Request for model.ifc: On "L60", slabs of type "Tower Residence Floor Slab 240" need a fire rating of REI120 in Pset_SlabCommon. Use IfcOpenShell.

First a look at what the model holds.

```python
import ifcopenshell
import ifcopenshell.util.element

model = ifcopenshell.open("model.ifc")
print(model.schema)
storey = next(s for s in model.by_type("IfcBuildingStorey") if s.Name == "L60")
slabs = [e for e in ifcopenshell.util.element.get_decomposition(storey) if e.is_a("IfcSlab")]
seen = {}
for e in slabs:
    element_type = ifcopenshell.util.element.get_type(e)
    key = (element_type.Name if element_type != e and element_type else None, ifcopenshell.util.element.get_pset(e, "Pset_SlabCommon", "FireRating"))
    seen[key] = seen.get(key, 0) + 1
for (name, value), count in sorted(seen.items(), key=str):
    print(count, "x", name, "|", value)
```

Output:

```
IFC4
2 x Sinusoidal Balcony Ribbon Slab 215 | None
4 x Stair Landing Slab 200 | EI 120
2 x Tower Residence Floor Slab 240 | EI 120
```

```python
import ifcopenshell
import ifcopenshell.api.pset
import ifcopenshell.util.element

model = ifcopenshell.open("model.ifc")

storey = next(s for s in model.by_type("IfcBuildingStorey") if s.Name == "L60")
slabs = [e for e in ifcopenshell.util.element.get_decomposition(storey) if e.is_a("IfcSlab")]

count = 0
for e in slabs:
    element_type = ifcopenshell.util.element.get_type(e)
    if element_type in (None, e) or element_type.Name != "Tower Residence Floor Slab 240":
        continue
    found = ifcopenshell.util.element.get_pset(e, "Pset_SlabCommon", should_inherit=False)
    if found:
        pset = model.by_id(found["id"])
        if len(ifcopenshell.util.element.get_elements_by_pset(pset)) > 1:
            pset = ifcopenshell.api.pset.unshare_pset(model, products=[e], pset=pset)[0]
    else:
        pset = ifcopenshell.api.pset.add_pset(model, product=e, name="Pset_SlabCommon")
    ifcopenshell.api.pset.edit_pset(model, pset=pset, properties={"FireRating": "REI120"})
    count += 1

print(count, "slabs updated")

model.write("model_v2.ifc")
```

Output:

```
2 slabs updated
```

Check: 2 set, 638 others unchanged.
